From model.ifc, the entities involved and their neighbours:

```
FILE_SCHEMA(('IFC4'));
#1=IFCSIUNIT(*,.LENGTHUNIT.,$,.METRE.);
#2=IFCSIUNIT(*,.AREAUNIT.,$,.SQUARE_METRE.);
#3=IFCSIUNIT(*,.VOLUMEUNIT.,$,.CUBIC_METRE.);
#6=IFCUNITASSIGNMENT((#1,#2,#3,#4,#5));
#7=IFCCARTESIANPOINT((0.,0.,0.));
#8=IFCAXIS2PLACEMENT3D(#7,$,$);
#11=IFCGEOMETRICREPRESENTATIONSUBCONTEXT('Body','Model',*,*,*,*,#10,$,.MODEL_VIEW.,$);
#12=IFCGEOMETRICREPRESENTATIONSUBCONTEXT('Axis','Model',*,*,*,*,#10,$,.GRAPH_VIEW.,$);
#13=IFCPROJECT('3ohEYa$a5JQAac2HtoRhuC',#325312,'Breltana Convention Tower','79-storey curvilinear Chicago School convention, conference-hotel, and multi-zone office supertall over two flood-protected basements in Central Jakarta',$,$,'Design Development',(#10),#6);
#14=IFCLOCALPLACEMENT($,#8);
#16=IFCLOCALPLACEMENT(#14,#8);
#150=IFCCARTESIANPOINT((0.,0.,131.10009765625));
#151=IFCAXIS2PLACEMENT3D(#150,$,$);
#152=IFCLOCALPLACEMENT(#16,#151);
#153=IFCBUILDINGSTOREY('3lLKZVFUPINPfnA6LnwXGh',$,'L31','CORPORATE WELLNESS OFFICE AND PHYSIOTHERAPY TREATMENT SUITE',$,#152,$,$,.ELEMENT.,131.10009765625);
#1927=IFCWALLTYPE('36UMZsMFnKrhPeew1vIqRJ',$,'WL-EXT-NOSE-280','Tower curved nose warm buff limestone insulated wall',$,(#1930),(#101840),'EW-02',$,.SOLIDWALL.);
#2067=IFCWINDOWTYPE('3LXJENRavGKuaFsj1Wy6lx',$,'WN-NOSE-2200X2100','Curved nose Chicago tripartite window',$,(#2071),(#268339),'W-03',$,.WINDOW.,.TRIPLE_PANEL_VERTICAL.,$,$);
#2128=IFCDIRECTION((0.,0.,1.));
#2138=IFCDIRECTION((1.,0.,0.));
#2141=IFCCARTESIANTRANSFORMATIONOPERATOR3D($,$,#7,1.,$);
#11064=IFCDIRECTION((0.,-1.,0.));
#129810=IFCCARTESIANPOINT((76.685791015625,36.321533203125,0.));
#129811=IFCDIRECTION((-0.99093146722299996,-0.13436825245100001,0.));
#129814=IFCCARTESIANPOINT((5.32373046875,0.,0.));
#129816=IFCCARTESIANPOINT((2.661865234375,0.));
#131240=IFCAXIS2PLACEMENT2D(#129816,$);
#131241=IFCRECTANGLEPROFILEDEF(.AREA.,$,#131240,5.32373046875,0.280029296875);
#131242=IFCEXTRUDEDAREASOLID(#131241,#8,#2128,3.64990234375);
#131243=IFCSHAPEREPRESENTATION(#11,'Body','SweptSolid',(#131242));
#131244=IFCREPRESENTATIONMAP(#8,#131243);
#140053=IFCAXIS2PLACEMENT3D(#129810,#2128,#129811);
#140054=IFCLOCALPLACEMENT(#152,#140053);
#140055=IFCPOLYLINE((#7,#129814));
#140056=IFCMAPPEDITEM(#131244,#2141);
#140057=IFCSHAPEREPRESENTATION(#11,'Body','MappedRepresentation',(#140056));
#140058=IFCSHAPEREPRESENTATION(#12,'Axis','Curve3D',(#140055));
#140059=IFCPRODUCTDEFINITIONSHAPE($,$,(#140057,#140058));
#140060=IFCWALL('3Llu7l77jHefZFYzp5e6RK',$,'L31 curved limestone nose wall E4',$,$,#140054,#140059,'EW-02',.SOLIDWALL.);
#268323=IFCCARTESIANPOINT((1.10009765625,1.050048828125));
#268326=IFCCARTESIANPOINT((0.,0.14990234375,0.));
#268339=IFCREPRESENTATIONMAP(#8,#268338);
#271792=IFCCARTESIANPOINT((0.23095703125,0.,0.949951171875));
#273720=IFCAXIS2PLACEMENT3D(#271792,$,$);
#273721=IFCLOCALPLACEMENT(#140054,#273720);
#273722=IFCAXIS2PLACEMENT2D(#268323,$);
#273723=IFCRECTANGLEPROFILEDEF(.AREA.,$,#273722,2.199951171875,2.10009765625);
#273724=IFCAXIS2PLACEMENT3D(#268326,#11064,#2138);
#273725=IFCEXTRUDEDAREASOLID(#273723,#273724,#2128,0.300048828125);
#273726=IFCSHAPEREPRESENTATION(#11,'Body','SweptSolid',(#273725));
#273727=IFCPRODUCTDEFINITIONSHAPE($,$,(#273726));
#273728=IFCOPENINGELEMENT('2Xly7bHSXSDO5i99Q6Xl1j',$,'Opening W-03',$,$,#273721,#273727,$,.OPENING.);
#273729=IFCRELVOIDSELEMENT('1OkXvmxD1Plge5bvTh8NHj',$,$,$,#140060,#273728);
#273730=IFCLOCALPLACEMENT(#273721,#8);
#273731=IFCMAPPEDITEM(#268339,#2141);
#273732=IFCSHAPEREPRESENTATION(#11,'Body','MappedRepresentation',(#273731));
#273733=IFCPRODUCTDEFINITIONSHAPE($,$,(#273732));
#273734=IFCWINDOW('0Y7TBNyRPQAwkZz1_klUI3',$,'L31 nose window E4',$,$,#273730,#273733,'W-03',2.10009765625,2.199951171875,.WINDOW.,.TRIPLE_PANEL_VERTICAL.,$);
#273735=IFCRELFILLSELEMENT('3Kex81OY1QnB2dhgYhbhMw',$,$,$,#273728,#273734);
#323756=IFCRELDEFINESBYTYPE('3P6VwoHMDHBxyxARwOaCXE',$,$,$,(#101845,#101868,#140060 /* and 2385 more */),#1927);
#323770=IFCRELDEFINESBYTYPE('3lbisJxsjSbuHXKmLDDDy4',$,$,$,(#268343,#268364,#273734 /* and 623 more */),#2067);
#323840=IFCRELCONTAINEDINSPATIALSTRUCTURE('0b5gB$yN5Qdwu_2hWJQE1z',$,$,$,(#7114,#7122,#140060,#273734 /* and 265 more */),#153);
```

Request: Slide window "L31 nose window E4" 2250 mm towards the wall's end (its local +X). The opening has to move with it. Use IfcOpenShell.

```python
import ifcopenshell
import ifcopenshell.api.geometry
import ifcopenshell.util.placement
import ifcopenshell.util.unit

model = ifcopenshell.open("model.ifc")
unit_scale = ifcopenshell.util.unit.calculate_unit_scale(model)

window = model.by_guid("0Y7TBNyRPQAwkZz1_klUI3")
opening = window.FillsVoids[0].RelatingOpeningElement
wall = opening.VoidsElements[0].RelatingBuildingElement

wall_matrix = ifcopenshell.util.placement.get_local_placement(wall.ObjectPlacement)
shift = wall_matrix[:3, 0] * 2.25 / unit_scale
before = ifcopenshell.util.placement.get_local_placement(window.ObjectPlacement)[:3, 3].copy()

# The window is placed relative to its opening, so it follows when the opening moves.
matrix = ifcopenshell.util.placement.get_local_placement(opening.ObjectPlacement)
matrix[:3, 3] += shift
ifcopenshell.api.geometry.edit_object_placement(
    model, product=opening, matrix=matrix, is_si=False, should_transform_children=True
)

after = ifcopenshell.util.placement.get_local_placement(window.ObjectPlacement)[:3, 3]
print("window moved by", (after - before).round(3) + 0.0)

model.write("model_rev.ifc")
```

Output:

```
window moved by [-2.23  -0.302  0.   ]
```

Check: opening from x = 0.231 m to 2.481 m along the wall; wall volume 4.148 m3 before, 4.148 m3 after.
